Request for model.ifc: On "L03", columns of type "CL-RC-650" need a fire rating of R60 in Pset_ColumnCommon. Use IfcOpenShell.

First a look at what the model holds.

```python
import ifcopenshell
import ifcopenshell.util.element

model = ifcopenshell.open("model.ifc")
print(model.schema)
storey = next(s for s in model.by_type("IfcBuildingStorey") if s.Name == "L03")
columns = [e for e in ifcopenshell.util.element.get_decomposition(storey) if e.is_a("IfcColumn")]
seen = {}
for e in columns:
    element_type = ifcopenshell.util.element.get_type(e)
    key = (element_type.Name if element_type != e and element_type else None, ifcopenshell.util.element.get_pset(e, "Pset_ColumnCommon", "FireRating"))
    seen[key] = seen.get(key, 0) + 1
for (name, value), count in sorted(seen.items(), key=str):
    print(count, "x", name, "|", value)
```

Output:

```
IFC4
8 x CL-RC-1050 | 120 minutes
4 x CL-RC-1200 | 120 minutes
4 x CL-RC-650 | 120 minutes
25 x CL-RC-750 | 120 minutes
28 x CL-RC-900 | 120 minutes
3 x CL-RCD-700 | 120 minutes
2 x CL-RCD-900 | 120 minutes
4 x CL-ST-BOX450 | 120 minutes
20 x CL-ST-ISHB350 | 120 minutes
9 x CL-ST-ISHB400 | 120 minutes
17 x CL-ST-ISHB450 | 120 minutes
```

```python
import ifcopenshell
import ifcopenshell.api.pset
import ifcopenshell.util.element

model = ifcopenshell.open("model.ifc")

storey = next(s for s in model.by_type("IfcBuildingStorey") if s.Name == "L03")
columns = [e for e in ifcopenshell.util.element.get_decomposition(storey) if e.is_a("IfcColumn")]

count = 0
for e in columns:
    element_type = ifcopenshell.util.element.get_type(e)
    if element_type in (None, e) or element_type.Name != "CL-RC-650":
        continue
    # add_pset returns the element's existing set when there is one.
    pset = ifcopenshell.api.pset.add_pset(model, product=e, name="Pset_ColumnCommon")
    ifcopenshell.api.pset.edit_pset(model, pset=pset, properties={"FireRating": "R60"})
    count += 1

print(count, "columns updated")

model.write("model_updated.ifc")
```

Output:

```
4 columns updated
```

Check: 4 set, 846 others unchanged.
